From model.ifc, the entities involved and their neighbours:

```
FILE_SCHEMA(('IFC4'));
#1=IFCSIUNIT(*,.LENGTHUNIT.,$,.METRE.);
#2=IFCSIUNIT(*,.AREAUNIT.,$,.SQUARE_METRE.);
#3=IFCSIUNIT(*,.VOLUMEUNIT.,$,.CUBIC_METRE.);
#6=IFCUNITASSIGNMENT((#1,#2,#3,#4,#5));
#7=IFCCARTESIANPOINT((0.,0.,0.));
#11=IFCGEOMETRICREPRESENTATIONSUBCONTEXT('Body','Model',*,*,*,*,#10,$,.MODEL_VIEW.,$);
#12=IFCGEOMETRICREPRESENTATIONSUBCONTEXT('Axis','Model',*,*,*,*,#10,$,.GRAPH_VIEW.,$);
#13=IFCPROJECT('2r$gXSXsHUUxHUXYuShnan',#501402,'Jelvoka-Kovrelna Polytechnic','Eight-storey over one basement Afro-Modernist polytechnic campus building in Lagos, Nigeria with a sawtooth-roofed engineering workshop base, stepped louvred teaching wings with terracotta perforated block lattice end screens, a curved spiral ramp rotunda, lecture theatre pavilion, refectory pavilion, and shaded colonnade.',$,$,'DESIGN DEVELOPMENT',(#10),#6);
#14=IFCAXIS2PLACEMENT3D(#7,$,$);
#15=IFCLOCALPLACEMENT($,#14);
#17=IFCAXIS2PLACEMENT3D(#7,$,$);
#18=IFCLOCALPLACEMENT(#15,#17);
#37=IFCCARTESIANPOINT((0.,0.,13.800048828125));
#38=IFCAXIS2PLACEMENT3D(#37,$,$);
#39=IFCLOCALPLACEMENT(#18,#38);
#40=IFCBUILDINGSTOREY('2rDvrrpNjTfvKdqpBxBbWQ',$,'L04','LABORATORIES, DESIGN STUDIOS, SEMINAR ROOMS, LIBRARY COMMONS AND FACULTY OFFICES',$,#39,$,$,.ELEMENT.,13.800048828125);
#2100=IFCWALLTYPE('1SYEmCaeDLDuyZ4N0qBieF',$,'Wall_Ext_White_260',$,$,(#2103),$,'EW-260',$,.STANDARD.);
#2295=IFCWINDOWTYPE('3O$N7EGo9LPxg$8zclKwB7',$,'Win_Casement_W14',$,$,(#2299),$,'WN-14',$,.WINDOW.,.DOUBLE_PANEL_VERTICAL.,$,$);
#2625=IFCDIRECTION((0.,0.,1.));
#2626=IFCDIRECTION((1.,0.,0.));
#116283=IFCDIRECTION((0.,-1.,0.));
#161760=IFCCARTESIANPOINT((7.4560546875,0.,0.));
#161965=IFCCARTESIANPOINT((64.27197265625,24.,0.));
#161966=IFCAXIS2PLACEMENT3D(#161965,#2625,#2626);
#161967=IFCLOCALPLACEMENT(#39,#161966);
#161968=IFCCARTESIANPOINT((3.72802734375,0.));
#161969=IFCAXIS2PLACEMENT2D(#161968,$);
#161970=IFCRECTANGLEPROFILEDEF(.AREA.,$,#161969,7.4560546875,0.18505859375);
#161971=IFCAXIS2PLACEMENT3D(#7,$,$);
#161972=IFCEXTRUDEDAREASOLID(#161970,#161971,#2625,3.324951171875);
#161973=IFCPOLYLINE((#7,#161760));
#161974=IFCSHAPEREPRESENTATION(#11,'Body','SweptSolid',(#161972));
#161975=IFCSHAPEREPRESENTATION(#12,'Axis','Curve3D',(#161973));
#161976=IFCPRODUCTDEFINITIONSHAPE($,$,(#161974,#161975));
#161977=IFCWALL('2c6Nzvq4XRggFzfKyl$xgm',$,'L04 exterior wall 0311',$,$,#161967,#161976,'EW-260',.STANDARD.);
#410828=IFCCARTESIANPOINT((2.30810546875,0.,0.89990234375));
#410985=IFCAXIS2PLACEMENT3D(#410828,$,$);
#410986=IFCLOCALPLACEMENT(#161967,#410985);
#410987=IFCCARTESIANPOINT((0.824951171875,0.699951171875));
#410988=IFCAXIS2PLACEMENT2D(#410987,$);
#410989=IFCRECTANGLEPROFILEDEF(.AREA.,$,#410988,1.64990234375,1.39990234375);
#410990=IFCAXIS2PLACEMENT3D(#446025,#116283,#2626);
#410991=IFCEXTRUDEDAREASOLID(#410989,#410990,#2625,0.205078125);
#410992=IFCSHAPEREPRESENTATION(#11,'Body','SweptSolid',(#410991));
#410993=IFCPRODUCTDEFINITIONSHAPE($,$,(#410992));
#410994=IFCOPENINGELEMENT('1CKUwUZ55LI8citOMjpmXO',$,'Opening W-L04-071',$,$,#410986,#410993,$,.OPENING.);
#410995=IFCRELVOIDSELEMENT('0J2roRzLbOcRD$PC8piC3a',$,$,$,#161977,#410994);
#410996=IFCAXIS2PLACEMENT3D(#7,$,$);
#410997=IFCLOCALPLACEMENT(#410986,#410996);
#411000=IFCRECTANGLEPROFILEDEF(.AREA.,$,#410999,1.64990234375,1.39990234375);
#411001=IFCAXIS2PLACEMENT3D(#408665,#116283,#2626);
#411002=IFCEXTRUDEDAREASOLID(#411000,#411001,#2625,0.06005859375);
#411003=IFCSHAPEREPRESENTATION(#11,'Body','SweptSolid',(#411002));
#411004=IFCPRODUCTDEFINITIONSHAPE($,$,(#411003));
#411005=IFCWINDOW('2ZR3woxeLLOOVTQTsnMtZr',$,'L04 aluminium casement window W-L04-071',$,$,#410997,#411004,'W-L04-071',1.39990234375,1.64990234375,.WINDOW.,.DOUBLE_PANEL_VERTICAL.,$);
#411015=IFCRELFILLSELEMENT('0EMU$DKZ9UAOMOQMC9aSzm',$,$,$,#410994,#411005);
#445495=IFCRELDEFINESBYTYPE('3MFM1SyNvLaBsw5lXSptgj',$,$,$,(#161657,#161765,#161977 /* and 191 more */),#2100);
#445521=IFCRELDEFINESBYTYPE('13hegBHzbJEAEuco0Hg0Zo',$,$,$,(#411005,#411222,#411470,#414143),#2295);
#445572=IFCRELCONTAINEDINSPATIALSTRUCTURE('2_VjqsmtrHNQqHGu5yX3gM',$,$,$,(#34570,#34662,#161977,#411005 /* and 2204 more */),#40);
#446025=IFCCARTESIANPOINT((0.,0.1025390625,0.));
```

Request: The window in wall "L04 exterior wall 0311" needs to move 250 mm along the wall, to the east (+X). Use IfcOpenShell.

```python
import ifcopenshell
import ifcopenshell.api.geometry
import ifcopenshell.util.placement
import ifcopenshell.util.unit

model = ifcopenshell.open("model.ifc")
unit_scale = ifcopenshell.util.unit.calculate_unit_scale(model)

window = model.by_guid("2ZR3woxeLLOOVTQTsnMtZr")
opening = window.FillsVoids[0].RelatingOpeningElement
wall = opening.VoidsElements[0].RelatingBuildingElement

wall_matrix = ifcopenshell.util.placement.get_local_placement(wall.ObjectPlacement)
shift = wall_matrix[:3, 0] * 0.25 / unit_scale
before = ifcopenshell.util.placement.get_local_placement(window.ObjectPlacement)[:3, 3].copy()

# The window is placed relative to its opening, so it follows when the opening moves.
matrix = ifcopenshell.util.placement.get_local_placement(opening.ObjectPlacement)
matrix[:3, 3] += shift
ifcopenshell.api.geometry.edit_object_placement(
    model, product=opening, matrix=matrix, is_si=False, should_transform_children=True
)

after = ifcopenshell.util.placement.get_local_placement(window.ObjectPlacement)[:3, 3]
print("window moved by", (after - before).round(3) + 0.0)

model.write("model_edited.ifc")
```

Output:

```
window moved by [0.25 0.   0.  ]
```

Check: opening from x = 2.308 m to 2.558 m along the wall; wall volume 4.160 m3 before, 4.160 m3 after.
